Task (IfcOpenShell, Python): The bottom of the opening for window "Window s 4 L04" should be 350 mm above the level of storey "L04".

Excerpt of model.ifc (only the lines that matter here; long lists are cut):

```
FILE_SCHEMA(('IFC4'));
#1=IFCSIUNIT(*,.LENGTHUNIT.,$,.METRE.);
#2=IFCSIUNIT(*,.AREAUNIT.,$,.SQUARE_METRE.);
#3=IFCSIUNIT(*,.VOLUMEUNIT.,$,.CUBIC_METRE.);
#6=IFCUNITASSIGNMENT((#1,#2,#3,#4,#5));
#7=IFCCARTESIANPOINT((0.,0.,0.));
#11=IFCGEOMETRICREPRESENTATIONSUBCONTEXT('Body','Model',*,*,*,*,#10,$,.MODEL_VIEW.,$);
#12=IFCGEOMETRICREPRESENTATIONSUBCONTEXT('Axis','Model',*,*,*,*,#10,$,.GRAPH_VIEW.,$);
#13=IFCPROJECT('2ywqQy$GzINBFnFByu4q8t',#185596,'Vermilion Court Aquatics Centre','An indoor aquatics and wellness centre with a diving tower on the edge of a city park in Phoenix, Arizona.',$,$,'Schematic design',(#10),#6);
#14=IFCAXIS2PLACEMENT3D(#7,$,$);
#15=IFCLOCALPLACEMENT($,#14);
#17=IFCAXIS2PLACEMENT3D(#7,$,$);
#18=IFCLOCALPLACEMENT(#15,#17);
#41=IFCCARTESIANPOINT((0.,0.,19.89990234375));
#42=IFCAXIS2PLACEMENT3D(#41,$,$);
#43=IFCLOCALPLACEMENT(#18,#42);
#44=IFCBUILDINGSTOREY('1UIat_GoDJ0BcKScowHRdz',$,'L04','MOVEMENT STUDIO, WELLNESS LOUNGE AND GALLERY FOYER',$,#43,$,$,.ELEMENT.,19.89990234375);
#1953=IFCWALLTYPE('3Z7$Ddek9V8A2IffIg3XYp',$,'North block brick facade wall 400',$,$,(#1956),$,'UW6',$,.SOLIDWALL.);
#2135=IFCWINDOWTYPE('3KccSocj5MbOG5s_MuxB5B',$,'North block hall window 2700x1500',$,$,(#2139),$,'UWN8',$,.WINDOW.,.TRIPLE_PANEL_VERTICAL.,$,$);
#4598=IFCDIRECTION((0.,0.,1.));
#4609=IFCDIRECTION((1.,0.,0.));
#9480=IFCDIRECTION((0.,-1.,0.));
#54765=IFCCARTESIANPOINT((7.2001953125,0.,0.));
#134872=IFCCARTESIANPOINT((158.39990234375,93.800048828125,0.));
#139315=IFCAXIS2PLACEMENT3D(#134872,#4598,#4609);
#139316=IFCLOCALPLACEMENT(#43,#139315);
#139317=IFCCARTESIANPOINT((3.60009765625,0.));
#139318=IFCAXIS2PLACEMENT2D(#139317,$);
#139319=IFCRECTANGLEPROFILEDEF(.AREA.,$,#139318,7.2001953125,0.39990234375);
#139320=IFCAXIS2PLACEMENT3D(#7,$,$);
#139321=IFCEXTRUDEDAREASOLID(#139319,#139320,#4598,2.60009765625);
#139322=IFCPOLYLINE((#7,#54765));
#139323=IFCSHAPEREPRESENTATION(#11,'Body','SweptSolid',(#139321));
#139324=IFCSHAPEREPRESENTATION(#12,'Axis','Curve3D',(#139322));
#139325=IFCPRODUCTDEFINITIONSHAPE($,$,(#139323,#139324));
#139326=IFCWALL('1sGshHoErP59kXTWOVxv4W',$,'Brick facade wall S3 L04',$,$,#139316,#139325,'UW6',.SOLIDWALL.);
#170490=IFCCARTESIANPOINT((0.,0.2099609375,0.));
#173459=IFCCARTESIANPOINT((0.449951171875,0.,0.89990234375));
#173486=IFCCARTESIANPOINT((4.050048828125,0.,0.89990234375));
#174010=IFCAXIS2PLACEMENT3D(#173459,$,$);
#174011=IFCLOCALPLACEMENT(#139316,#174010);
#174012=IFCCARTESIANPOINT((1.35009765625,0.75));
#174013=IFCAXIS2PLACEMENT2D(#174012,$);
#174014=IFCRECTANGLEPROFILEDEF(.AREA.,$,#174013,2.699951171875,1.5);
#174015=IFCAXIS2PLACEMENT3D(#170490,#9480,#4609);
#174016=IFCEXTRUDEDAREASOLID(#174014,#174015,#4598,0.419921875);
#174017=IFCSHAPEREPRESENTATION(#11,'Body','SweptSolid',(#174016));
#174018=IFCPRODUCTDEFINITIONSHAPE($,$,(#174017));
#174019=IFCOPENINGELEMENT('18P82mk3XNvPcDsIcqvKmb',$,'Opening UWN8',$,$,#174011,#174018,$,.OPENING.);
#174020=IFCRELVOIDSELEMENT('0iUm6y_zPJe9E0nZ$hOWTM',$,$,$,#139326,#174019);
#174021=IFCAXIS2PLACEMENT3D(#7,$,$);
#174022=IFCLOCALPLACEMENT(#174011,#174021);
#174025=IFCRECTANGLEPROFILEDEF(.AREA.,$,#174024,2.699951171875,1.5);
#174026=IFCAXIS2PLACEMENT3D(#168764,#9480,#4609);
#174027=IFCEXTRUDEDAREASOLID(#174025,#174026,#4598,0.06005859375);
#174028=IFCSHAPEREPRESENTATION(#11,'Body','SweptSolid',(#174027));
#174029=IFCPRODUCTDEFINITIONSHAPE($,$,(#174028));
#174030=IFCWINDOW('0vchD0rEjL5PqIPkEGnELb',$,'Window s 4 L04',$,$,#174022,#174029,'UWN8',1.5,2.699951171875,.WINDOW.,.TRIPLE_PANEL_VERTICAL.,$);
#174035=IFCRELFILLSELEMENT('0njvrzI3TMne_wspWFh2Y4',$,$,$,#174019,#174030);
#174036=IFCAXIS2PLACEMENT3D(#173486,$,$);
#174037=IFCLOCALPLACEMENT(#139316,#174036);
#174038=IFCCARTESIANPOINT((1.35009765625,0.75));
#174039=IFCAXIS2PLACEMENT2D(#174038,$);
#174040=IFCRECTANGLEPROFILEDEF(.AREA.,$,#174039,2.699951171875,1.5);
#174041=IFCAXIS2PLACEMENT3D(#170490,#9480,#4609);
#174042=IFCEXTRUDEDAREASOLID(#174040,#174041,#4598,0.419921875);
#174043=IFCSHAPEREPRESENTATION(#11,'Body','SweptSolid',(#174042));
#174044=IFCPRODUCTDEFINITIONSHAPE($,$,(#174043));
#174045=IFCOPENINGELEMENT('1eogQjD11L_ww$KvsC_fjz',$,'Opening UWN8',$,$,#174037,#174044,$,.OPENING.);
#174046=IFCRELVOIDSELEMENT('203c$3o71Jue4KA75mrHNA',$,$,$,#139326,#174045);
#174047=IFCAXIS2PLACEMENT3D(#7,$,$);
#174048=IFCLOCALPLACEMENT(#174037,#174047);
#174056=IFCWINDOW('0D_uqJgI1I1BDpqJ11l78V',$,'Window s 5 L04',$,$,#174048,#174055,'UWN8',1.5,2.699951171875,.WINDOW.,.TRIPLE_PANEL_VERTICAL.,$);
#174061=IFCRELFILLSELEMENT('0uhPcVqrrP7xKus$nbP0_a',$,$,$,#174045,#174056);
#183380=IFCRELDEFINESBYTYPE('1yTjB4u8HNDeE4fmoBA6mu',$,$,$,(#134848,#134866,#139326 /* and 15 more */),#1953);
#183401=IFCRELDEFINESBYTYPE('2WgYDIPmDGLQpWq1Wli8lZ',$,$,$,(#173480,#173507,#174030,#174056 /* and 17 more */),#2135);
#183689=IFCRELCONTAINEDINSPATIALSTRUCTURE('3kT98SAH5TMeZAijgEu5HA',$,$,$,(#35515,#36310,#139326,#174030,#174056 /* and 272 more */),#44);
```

```python
import numpy as np
import ifcopenshell
import ifcopenshell.api.geometry
import ifcopenshell.geom
import ifcopenshell.util.element
import ifcopenshell.util.placement
import ifcopenshell.util.shape
import ifcopenshell.util.unit

model = ifcopenshell.open("model.ifc")
unit_scale = ifcopenshell.util.unit.calculate_unit_scale(model)

window = model.by_guid("0vchD0rEjL5PqIPkEGnELb")
opening = window.FillsVoids[0].RelatingOpeningElement
storey = ifcopenshell.util.element.get_container(window, ifc_class="IfcBuildingStorey")
level = ifcopenshell.util.placement.get_local_placement(storey.ObjectPlacement)[2, 3]

# The opening's origin need not be at the sill, so measure its lowest point.
shape = ifcopenshell.geom.create_shape(ifcopenshell.geom.settings(), opening)
bottom = ifcopenshell.util.shape.get_shape_bottom_elevation(shape, shape.geometry) / unit_scale
dz = level + 0.35 / unit_scale - bottom

shift = np.array([0.0, 0.0, dz])
# The window is placed relative to its opening, so it follows when the opening moves.
matrix = ifcopenshell.util.placement.get_local_placement(opening.ObjectPlacement)
matrix[:3, 3] += shift
ifcopenshell.api.geometry.edit_object_placement(
    model, product=opening, matrix=matrix, is_si=False, should_transform_children=True
)

print(f"moved by {dz * unit_scale:+.3f} m")

model.write("model_v2.ifc")
```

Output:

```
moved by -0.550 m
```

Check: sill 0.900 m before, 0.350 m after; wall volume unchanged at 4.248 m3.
